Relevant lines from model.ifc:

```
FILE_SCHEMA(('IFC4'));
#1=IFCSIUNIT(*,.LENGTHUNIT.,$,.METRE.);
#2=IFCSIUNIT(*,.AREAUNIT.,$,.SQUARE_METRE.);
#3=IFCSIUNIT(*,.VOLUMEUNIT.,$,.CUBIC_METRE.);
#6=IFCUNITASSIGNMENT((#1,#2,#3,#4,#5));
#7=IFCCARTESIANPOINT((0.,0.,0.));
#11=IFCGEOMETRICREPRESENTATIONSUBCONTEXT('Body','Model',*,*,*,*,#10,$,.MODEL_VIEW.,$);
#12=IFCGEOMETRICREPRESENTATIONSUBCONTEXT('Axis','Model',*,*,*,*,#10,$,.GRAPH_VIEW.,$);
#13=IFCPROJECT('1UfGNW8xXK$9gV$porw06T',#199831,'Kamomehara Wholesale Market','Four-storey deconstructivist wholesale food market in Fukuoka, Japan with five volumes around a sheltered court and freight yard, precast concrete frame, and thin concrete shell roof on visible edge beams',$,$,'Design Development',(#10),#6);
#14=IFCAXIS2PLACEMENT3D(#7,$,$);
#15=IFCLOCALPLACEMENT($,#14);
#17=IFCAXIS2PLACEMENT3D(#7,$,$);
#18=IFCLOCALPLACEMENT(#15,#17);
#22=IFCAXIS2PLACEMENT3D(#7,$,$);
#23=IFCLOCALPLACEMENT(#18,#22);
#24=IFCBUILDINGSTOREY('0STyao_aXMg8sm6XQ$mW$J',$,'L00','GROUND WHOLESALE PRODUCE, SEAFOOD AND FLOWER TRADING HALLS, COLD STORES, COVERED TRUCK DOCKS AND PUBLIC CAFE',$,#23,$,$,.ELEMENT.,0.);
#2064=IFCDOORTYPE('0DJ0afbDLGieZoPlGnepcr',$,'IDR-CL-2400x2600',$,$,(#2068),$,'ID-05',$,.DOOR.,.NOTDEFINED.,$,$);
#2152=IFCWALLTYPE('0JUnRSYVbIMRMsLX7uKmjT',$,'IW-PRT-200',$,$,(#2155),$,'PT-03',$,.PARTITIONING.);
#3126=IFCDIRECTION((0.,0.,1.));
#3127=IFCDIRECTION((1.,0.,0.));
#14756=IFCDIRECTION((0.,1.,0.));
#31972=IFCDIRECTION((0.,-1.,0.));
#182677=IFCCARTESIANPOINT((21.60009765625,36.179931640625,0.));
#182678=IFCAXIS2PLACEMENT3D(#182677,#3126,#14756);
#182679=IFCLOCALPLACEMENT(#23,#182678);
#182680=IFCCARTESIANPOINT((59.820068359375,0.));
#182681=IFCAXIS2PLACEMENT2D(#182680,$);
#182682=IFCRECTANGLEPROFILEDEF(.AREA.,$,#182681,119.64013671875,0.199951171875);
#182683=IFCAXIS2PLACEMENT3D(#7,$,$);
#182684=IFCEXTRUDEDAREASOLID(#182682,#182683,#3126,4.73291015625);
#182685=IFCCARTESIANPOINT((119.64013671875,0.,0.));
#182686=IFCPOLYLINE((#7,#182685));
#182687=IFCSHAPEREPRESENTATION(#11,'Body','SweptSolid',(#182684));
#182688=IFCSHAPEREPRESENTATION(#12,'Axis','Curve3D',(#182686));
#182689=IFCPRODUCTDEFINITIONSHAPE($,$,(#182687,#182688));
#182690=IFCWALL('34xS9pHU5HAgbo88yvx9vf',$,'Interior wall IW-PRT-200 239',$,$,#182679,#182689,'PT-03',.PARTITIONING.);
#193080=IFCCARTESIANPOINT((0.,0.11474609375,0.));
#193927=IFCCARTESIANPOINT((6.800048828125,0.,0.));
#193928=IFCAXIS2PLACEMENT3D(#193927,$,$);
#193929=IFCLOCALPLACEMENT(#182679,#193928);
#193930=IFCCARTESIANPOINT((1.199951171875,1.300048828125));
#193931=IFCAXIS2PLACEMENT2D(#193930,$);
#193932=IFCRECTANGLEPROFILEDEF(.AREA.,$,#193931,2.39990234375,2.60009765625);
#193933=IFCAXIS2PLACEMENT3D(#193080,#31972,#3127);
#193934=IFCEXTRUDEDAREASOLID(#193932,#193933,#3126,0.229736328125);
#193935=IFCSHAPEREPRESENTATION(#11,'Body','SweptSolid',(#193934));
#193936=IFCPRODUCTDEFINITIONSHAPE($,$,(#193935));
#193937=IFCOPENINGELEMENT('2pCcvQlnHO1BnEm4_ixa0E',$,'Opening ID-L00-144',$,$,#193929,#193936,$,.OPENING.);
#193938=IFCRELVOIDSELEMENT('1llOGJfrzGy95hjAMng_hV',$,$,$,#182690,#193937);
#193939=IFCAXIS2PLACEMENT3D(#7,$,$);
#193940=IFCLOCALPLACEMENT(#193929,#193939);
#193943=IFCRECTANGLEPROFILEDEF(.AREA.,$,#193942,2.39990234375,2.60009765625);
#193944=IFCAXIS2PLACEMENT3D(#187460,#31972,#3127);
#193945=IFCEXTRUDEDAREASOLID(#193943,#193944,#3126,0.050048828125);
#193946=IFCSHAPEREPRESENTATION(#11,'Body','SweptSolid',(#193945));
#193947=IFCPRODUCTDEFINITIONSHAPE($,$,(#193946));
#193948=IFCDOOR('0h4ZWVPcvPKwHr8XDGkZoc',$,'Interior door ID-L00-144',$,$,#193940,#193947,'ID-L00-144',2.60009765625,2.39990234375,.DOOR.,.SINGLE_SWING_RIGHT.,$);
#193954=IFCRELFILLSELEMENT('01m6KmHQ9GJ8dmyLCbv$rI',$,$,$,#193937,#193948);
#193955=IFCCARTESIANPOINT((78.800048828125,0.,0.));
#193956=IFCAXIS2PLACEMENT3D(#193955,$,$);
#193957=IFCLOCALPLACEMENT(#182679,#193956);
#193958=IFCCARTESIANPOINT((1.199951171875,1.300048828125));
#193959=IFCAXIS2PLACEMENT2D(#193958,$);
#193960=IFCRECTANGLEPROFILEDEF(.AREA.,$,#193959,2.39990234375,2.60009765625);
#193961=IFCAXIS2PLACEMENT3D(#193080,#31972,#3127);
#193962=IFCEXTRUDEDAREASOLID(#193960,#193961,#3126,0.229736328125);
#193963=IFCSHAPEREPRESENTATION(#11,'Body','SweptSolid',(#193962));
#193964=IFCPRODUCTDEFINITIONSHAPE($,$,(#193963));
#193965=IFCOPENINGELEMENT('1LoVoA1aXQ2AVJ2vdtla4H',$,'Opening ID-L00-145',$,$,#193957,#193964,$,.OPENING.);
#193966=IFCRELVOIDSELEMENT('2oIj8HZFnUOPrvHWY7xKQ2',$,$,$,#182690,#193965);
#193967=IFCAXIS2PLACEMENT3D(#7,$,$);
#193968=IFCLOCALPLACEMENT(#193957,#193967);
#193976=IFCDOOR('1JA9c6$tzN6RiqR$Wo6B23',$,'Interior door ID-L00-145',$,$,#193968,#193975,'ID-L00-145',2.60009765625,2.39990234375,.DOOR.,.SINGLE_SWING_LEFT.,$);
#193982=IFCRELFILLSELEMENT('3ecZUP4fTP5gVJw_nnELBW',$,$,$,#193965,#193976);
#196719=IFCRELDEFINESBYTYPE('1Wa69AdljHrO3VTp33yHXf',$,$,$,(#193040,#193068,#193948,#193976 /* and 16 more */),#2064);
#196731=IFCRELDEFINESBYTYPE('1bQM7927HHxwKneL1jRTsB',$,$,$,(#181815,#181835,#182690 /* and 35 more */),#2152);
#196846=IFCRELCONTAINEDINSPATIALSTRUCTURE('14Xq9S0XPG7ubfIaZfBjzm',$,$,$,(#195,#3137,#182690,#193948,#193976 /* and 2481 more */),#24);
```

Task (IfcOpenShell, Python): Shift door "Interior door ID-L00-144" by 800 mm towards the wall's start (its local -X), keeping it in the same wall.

```python
import ifcopenshell
import ifcopenshell.api.geometry
import ifcopenshell.util.placement
import ifcopenshell.util.unit

model = ifcopenshell.open("model.ifc")
unit_scale = ifcopenshell.util.unit.calculate_unit_scale(model)

door = model.by_guid("0h4ZWVPcvPKwHr8XDGkZoc")
opening = door.FillsVoids[0].RelatingOpeningElement
wall = opening.VoidsElements[0].RelatingBuildingElement

wall_matrix = ifcopenshell.util.placement.get_local_placement(wall.ObjectPlacement)
shift = wall_matrix[:3, 0] * -0.8 / unit_scale
before = ifcopenshell.util.placement.get_local_placement(door.ObjectPlacement)[:3, 3].copy()

# The door is placed relative to its opening, so it follows when the opening moves.
matrix = ifcopenshell.util.placement.get_local_placement(opening.ObjectPlacement)
matrix[:3, 3] += shift
ifcopenshell.api.geometry.edit_object_placement(
    model, product=opening, matrix=matrix, is_si=False, should_transform_children=True
)

after = ifcopenshell.util.placement.get_local_placement(door.ObjectPlacement)[:3, 3]
print("door moved by", (after - before).round(3) + 0.0)

model.write("model_v2.ifc")
```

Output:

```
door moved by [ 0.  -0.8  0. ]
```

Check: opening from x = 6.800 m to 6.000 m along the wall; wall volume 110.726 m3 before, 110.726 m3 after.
